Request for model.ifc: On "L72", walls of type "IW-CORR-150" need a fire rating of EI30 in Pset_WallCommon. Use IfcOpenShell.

First a look at what the model holds.

```python
import ifcopenshell
import ifcopenshell.util.element

model = ifcopenshell.open("model.ifc")
print(model.schema)
storey = next(s for s in model.by_type("IfcBuildingStorey") if s.Name == "L72")
walls = [e for e in ifcopenshell.util.element.get_decomposition(storey) if e.is_a("IfcWall")]
seen = {}
for e in walls:
    element_type = ifcopenshell.util.element.get_type(e)
    key = (element_type.Name if element_type != e and element_type else None, ifcopenshell.util.element.get_pset(e, "Pset_WallCommon", "FireRating"))
    seen[key] = seen.get(key, 0) + 1
for (name, value), count in sorted(seen.items(), key=str):
    print(count, "x", name, "|", value)
```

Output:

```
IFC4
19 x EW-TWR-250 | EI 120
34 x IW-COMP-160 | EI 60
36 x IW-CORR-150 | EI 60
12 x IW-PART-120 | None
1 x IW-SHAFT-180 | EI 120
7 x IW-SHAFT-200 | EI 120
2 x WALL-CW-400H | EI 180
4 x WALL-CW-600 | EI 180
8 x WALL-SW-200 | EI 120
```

```python
import ifcopenshell
import ifcopenshell.api.pset
import ifcopenshell.util.element

model = ifcopenshell.open("model.ifc")

storey = next(s for s in model.by_type("IfcBuildingStorey") if s.Name == "L72")
walls = [e for e in ifcopenshell.util.element.get_decomposition(storey) if e.is_a("IfcWall")]

count = 0
for e in walls:
    element_type = ifcopenshell.util.element.get_type(e)
    if element_type in (None, e) or element_type.Name != "IW-CORR-150":
        continue
    found = ifcopenshell.util.element.get_pset(e, "Pset_WallCommon", should_inherit=False)
    if found:
        pset = model.by_id(found["id"])
        if len(ifcopenshell.util.element.get_elements_by_pset(pset)) > 1:
            pset = ifcopenshell.api.pset.unshare_pset(model, products=[e], pset=pset)[0]
    else:
        pset = ifcopenshell.api.pset.add_pset(model, product=e, name="Pset_WallCommon")
    ifcopenshell.api.pset.edit_pset(model, pset=pset, properties={"FireRating": "EI30"})
    count += 1

print(count, "walls updated")

model.write("model_edited.ifc")
```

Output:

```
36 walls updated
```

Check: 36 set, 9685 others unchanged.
